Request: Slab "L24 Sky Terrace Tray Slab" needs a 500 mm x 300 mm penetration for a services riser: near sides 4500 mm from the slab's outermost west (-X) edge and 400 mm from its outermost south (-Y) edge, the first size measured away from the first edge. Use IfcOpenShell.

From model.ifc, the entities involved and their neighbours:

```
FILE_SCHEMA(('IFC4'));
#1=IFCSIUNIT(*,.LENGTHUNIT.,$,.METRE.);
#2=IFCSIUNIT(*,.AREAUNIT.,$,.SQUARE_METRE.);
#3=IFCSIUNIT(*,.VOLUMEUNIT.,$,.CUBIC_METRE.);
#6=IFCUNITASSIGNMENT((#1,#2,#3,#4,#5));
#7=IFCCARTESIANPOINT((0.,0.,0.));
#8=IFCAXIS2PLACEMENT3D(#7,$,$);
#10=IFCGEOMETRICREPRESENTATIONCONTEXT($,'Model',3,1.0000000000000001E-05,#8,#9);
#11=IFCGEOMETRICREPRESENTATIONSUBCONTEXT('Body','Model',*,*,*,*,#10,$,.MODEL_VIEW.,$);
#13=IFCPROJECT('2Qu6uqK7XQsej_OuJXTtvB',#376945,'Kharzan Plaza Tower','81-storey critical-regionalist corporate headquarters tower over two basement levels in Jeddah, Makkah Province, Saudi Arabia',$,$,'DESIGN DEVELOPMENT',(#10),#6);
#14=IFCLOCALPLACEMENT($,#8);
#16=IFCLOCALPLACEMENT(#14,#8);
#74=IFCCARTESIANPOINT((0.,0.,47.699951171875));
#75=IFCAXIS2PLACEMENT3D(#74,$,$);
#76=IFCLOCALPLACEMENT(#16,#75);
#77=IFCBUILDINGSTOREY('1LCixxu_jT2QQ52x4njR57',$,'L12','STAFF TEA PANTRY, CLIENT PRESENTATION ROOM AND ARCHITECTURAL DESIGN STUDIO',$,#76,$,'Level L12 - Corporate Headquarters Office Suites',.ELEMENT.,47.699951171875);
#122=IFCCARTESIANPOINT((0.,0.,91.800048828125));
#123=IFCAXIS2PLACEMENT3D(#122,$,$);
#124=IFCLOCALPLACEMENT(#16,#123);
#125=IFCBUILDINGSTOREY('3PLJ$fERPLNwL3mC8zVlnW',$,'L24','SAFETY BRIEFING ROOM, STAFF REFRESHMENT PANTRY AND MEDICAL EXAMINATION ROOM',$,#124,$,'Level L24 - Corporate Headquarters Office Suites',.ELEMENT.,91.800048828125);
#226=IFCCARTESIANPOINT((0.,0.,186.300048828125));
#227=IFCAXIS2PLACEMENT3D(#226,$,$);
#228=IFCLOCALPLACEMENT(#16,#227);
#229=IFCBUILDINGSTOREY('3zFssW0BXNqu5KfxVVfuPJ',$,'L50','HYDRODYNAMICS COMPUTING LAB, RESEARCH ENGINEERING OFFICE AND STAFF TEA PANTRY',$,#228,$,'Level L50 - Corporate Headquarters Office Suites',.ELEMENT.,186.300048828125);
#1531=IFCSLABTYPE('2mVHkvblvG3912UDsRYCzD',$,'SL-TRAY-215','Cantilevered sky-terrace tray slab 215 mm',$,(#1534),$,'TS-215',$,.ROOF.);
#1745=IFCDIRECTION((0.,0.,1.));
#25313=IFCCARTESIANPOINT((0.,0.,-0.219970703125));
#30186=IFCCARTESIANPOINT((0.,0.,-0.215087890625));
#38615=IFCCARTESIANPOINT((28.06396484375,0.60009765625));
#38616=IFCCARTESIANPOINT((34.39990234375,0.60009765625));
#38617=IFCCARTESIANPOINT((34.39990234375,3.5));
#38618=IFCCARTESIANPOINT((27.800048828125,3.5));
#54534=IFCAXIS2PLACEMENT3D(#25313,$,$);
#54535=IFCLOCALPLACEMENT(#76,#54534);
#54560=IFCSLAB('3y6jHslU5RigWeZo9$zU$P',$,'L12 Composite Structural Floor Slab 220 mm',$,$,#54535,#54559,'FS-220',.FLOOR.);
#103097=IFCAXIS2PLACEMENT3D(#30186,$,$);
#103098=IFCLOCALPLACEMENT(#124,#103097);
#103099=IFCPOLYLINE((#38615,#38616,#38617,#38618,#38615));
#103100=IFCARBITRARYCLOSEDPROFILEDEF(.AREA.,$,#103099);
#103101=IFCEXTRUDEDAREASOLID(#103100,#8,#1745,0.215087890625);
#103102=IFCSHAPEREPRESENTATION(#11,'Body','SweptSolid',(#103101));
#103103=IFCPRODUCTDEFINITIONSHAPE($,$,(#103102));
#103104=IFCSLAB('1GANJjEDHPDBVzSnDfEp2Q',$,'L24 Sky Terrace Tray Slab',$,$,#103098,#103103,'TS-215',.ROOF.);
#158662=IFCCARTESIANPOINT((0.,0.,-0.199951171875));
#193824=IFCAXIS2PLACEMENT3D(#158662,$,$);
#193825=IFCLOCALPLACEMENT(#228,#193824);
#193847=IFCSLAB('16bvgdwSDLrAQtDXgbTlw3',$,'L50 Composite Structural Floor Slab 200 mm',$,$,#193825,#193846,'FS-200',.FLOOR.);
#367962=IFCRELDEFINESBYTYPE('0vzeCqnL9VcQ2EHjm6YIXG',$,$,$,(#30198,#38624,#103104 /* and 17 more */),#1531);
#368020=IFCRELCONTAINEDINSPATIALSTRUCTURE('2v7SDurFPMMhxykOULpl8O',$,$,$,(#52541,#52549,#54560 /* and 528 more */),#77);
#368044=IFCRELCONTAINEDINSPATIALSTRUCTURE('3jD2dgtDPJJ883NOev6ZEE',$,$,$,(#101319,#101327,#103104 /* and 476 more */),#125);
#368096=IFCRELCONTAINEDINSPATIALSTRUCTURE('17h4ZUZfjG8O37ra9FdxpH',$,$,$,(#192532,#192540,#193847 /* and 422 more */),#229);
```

```python
import numpy as np
import ifcopenshell
import ifcopenshell.api.feature
import ifcopenshell.api.geometry
import ifcopenshell.api.root
import ifcopenshell.geom
import ifcopenshell.util.placement
import ifcopenshell.util.representation
import ifcopenshell.util.shape
import ifcopenshell.util.unit

model = ifcopenshell.open("model.ifc")
unit_scale = ifcopenshell.util.unit.calculate_unit_scale(model)
settings = ifcopenshell.geom.settings()


def volume(element):
    """Net volume in cubic metres, openings subtracted."""
    shape = ifcopenshell.geom.create_shape(settings, element)
    return ifcopenshell.util.shape.get_volume(shape.geometry)


slab = model.by_guid("1GANJjEDHPDBVzSnDfEp2Q")
before = volume(slab)

# Extent in the slab's own axes, in metres. The edges named are its -X and -Y sides.
slab_shape = ifcopenshell.geom.create_shape(settings, slab)
vertices = ifcopenshell.util.shape.get_vertices(slab_shape.geometry)
x_min, y_min, bottom = vertices.min(axis=0)
top = vertices[:, 2].max()

opening = ifcopenshell.api.root.create_entity(model, ifc_class="IfcOpeningElement", name="Services riser opening", predefined_type="OPENING")
context = ifcopenshell.util.representation.get_context(model, "Model", "Body", "MODEL_VIEW")
width, depth = 0.5, 0.3
outline = [(0.0, 0.0), (width, 0.0), (width, depth), (0.0, depth), (0.0, 0.0)]
# Overshoot both faces by 50 mm so the cut is clean.
shape = ifcopenshell.api.geometry.add_slab_representation(
    model, context=context, depth=top - bottom + 0.1, polyline=outline
)
ifcopenshell.api.geometry.assign_representation(model, product=opening, representation=shape)

matrix = ifcopenshell.util.placement.get_local_placement(slab.ObjectPlacement)
matrix[:, 3] = matrix @ np.append(np.array([x_min + 4.5, y_min + 0.4, bottom - 0.05]) / unit_scale, 1.0)
ifcopenshell.api.geometry.edit_object_placement(model, product=opening, matrix=matrix, is_si=False)
ifcopenshell.api.feature.add_feature(model, feature=opening, element=slab)

after = volume(slab)

print(f"slab volume {before:.3f} -> {after:.3f} m3")

model.write("model_v2.ifc")
```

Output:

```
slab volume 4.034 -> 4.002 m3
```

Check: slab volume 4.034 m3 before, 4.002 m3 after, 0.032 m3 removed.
